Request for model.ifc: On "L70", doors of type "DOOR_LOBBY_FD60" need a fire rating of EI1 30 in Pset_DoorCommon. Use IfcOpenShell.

First a look at what the model holds.

```python
import ifcopenshell
import ifcopenshell.util.element

model = ifcopenshell.open("model.ifc")
print(model.schema)
storey = next(s for s in model.by_type("IfcBuildingStorey") if s.Name == "L70")
doors = [e for e in ifcopenshell.util.element.get_decomposition(storey) if e.is_a("IfcDoor")]
seen = {}
for e in doors:
    element_type = ifcopenshell.util.element.get_type(e)
    key = (element_type.Name if element_type != e and element_type else None, ifcopenshell.util.element.get_pset(e, "Pset_DoorCommon", "FireRating"))
    seen[key] = seen.get(key, 0) + 1
for (name, value), count in sorted(seen.items(), key=str):
    print(count, "x", name, "|", value)
```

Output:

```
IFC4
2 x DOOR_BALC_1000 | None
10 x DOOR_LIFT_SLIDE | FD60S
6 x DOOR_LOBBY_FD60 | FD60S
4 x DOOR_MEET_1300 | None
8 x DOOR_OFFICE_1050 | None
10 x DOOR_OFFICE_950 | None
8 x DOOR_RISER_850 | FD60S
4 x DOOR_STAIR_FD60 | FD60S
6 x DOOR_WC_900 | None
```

```python
import ifcopenshell
import ifcopenshell.api.pset
import ifcopenshell.util.element

model = ifcopenshell.open("model.ifc")

storey = next(s for s in model.by_type("IfcBuildingStorey") if s.Name == "L70")
doors = [e for e in ifcopenshell.util.element.get_decomposition(storey) if e.is_a("IfcDoor")]

count = 0
for e in doors:
    element_type = ifcopenshell.util.element.get_type(e)
    if element_type in (None, e) or element_type.Name != "DOOR_LOBBY_FD60":
        continue
    # add_pset returns the element's existing set when there is one.
    pset = ifcopenshell.api.pset.add_pset(model, product=e, name="Pset_DoorCommon")
    ifcopenshell.api.pset.edit_pset(model, pset=pset, properties={"FireRating": "EI1 30"})
    count += 1

print(count, "doors updated")

model.write("model_edited.ifc")
```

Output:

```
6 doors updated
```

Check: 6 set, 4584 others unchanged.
